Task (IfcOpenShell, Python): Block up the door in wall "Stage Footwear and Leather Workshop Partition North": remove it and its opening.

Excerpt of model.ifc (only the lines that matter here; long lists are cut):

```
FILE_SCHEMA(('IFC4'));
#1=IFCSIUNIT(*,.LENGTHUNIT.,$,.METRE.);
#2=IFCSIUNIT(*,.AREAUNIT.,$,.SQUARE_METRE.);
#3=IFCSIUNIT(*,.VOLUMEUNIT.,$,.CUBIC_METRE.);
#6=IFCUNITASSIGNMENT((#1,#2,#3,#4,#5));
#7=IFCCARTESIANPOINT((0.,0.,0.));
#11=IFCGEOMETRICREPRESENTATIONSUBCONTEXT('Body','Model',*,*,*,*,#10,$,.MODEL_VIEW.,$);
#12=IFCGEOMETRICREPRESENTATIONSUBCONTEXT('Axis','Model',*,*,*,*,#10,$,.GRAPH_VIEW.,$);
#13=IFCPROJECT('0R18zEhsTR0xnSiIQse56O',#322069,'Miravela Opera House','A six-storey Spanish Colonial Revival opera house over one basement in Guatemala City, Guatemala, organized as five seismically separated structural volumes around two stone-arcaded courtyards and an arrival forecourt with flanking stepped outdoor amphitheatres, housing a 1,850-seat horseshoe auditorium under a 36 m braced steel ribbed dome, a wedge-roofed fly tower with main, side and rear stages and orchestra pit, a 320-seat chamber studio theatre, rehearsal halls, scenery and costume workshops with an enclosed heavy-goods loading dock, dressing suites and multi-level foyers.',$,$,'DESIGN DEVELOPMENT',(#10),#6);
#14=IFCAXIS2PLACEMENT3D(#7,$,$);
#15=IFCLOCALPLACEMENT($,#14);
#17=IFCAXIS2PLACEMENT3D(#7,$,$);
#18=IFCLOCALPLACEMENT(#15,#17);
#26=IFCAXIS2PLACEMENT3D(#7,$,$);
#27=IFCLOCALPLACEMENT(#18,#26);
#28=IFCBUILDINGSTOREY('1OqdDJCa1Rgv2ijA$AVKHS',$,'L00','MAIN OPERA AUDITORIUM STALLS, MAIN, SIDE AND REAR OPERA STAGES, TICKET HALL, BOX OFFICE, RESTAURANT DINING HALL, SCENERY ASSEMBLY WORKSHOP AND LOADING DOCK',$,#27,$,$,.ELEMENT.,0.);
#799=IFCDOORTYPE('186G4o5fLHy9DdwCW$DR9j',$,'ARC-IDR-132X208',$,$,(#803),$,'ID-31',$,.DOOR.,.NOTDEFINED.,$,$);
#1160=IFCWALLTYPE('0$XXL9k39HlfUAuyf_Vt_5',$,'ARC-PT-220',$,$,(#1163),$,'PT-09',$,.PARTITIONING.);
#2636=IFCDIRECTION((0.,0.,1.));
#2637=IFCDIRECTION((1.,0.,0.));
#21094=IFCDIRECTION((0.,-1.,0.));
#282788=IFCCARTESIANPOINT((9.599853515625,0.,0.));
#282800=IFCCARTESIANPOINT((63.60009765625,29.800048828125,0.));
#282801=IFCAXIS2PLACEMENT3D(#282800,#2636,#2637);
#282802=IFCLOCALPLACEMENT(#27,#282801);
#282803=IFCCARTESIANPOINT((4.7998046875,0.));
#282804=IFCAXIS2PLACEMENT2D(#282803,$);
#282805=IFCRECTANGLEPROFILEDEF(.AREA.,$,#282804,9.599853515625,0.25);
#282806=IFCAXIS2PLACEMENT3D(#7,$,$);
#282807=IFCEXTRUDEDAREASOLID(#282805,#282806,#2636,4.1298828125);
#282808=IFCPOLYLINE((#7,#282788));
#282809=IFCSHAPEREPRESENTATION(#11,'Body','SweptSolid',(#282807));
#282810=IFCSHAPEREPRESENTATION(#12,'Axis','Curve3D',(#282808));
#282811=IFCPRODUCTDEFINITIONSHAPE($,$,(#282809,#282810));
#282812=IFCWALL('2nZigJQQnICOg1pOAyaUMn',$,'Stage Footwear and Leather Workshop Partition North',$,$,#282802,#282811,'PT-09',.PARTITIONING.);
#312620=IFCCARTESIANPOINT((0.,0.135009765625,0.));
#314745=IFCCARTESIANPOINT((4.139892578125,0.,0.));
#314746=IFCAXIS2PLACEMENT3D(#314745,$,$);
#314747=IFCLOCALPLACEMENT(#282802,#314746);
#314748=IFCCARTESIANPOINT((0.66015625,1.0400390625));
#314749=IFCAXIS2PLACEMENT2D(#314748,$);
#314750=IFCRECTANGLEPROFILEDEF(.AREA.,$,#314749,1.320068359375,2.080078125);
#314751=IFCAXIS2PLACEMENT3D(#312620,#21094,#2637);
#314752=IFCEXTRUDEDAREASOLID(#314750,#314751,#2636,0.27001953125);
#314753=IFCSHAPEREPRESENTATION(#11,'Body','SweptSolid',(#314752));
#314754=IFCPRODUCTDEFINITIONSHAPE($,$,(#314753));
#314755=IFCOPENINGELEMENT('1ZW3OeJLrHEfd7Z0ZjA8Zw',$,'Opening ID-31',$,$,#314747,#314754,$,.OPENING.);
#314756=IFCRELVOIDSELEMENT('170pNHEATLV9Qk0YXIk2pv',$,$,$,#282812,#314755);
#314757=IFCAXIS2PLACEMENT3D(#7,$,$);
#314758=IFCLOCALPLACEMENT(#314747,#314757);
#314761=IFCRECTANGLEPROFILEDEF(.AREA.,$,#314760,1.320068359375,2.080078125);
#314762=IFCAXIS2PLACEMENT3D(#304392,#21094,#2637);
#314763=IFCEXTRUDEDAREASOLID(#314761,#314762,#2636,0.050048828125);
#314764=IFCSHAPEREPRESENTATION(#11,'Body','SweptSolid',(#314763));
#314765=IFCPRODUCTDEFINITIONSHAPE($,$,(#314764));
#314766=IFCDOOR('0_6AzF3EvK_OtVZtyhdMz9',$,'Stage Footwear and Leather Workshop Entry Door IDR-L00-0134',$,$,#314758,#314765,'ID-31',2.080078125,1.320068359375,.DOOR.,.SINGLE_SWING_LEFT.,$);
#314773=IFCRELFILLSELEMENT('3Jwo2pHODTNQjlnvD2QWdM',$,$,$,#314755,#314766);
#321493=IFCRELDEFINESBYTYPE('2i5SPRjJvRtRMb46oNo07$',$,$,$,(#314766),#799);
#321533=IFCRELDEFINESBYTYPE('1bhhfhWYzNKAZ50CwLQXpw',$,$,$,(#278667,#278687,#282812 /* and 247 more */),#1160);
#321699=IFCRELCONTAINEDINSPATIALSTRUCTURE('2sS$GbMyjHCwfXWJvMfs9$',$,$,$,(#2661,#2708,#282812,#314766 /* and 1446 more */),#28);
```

```python
import ifcopenshell
import ifcopenshell.api.feature
import ifcopenshell.api.root
import ifcopenshell.geom
import ifcopenshell.util.shape

model = ifcopenshell.open("model.ifc")
settings = ifcopenshell.geom.settings()


def volume(element):
    """Net volume in cubic metres, openings subtracted."""
    shape = ifcopenshell.geom.create_shape(settings, element)
    return ifcopenshell.util.shape.get_volume(shape.geometry)


door = model.by_guid("0_6AzF3EvK_OtVZtyhdMz9")
opening = door.FillsVoids[0].RelatingOpeningElement
wall = opening.VoidsElements[0].RelatingBuildingElement
before = volume(wall)

ifcopenshell.api.root.remove_product(model, product=door)
ifcopenshell.api.feature.remove_feature(model, feature=opening)

after = volume(wall)

print(f"wall volume {before:.3f} -> {after:.3f} m3")

model.write("model_edited.ifc")
```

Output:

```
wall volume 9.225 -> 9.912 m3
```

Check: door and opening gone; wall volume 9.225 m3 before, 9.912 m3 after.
